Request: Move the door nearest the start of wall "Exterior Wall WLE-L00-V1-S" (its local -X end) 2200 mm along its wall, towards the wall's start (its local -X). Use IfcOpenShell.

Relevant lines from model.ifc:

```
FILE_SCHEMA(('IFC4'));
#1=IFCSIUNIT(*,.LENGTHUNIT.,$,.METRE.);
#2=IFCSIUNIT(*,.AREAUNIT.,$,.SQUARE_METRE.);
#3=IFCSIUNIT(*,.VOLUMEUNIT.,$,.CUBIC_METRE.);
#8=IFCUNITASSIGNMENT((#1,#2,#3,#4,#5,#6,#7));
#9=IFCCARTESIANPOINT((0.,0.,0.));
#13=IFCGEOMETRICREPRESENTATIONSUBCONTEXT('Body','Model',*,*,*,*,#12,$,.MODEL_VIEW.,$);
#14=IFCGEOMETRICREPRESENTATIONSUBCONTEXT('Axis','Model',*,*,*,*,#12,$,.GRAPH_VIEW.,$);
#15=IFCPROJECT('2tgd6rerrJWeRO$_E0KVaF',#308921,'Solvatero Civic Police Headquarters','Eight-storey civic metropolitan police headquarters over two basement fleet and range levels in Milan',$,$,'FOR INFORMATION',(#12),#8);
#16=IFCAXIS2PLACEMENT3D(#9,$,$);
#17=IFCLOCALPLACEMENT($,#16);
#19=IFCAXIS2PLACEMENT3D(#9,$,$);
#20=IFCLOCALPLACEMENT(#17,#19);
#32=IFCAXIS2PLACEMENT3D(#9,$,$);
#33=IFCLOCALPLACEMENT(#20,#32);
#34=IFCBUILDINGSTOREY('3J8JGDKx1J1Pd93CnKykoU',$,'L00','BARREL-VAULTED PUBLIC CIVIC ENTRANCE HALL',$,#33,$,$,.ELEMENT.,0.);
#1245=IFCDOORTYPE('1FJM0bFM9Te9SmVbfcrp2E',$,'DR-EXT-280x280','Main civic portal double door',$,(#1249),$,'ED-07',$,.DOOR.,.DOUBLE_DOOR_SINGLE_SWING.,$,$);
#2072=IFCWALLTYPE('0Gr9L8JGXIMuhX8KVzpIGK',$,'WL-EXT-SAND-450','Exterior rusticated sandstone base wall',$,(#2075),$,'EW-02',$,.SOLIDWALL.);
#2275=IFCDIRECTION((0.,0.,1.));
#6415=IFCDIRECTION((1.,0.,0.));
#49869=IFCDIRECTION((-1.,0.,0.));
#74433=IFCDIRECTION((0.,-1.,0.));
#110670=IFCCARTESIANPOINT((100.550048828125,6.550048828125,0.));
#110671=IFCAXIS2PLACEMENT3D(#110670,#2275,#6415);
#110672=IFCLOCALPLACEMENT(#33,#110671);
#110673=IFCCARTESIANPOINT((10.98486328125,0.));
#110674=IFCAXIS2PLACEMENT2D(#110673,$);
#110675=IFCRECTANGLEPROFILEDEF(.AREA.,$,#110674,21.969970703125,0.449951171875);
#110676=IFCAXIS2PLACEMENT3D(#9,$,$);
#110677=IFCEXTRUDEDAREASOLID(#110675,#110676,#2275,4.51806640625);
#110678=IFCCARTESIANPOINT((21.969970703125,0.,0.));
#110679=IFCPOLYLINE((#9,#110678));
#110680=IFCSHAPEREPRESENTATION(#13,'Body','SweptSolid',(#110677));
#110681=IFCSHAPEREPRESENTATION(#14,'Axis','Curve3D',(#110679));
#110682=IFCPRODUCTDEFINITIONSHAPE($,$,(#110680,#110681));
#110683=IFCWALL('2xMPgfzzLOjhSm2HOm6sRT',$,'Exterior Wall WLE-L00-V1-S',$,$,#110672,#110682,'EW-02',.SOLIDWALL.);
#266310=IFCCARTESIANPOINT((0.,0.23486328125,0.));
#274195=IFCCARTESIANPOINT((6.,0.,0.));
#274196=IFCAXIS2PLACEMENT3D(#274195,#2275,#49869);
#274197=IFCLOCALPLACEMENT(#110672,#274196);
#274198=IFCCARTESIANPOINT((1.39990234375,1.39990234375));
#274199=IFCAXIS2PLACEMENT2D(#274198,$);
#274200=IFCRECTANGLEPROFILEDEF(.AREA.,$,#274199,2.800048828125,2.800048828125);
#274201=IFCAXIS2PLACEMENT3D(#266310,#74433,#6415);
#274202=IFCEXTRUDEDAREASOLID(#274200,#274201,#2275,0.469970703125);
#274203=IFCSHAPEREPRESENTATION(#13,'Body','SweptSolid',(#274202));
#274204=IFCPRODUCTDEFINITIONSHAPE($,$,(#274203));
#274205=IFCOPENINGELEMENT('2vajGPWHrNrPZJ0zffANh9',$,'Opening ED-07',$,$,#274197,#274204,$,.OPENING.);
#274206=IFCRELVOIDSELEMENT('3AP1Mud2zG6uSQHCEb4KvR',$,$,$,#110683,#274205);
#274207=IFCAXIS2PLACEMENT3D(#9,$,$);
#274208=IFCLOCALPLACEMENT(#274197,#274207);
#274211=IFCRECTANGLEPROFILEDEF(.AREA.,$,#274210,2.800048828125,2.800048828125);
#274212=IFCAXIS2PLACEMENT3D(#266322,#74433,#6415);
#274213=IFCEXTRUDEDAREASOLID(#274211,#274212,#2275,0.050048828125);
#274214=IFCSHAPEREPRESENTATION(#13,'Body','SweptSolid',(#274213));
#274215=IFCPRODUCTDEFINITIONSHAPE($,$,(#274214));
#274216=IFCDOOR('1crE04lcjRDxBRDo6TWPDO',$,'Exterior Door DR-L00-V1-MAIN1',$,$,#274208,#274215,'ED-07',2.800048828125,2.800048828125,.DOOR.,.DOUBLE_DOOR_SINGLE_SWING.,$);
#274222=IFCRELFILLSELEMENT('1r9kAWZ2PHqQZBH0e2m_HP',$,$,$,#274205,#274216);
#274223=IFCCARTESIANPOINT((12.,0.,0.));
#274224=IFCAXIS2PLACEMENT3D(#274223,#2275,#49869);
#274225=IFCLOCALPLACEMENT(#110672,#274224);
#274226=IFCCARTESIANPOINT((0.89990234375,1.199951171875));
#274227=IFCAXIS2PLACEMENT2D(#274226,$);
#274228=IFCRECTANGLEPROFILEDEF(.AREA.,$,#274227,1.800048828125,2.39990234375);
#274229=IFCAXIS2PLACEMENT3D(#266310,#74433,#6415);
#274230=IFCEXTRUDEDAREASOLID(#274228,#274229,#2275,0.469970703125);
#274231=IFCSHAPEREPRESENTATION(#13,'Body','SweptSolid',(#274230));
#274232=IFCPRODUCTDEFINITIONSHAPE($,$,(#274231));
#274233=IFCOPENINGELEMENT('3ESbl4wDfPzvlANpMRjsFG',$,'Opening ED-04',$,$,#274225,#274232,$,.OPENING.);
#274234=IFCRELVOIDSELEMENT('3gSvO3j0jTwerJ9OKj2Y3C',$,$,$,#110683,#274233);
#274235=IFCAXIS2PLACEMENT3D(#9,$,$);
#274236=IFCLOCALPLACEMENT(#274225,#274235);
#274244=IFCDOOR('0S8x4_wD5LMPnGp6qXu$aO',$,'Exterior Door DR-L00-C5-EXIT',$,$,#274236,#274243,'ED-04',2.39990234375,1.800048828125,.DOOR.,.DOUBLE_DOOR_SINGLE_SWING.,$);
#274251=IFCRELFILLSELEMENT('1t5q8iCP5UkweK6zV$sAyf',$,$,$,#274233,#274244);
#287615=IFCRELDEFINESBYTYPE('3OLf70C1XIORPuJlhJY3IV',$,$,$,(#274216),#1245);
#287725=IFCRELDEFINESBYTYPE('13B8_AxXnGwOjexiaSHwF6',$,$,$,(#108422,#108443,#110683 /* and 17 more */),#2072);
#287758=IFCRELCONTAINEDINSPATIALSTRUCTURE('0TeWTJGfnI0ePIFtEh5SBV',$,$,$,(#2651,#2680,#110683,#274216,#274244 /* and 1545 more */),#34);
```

```python
import ifcopenshell
import ifcopenshell.api.geometry
import ifcopenshell.util.placement

model = ifcopenshell.open("model.ifc")

door = model.by_id(274216)
opening = door.FillsVoids[0].RelatingOpeningElement
wall = opening.VoidsElements[0].RelatingBuildingElement

wall_matrix = ifcopenshell.util.placement.get_local_placement(wall.ObjectPlacement)
shift = wall_matrix[:3, 0] * -2.2
before = ifcopenshell.util.placement.get_local_placement(door.ObjectPlacement)[:3, 3].copy()

# The door is placed relative to its opening, so it follows when the opening moves.
matrix = ifcopenshell.util.placement.get_local_placement(opening.ObjectPlacement)
matrix[:3, 3] += shift
ifcopenshell.api.geometry.edit_object_placement(
    model, product=opening, matrix=matrix, is_si=False, should_transform_children=True
)

after = ifcopenshell.util.placement.get_local_placement(door.ObjectPlacement)[:3, 3]
print("door moved by", (after - before).round(3) + 0.0)

model.write("model_updated.ifc")
```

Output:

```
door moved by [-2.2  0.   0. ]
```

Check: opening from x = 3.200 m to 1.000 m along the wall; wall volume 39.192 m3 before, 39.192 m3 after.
